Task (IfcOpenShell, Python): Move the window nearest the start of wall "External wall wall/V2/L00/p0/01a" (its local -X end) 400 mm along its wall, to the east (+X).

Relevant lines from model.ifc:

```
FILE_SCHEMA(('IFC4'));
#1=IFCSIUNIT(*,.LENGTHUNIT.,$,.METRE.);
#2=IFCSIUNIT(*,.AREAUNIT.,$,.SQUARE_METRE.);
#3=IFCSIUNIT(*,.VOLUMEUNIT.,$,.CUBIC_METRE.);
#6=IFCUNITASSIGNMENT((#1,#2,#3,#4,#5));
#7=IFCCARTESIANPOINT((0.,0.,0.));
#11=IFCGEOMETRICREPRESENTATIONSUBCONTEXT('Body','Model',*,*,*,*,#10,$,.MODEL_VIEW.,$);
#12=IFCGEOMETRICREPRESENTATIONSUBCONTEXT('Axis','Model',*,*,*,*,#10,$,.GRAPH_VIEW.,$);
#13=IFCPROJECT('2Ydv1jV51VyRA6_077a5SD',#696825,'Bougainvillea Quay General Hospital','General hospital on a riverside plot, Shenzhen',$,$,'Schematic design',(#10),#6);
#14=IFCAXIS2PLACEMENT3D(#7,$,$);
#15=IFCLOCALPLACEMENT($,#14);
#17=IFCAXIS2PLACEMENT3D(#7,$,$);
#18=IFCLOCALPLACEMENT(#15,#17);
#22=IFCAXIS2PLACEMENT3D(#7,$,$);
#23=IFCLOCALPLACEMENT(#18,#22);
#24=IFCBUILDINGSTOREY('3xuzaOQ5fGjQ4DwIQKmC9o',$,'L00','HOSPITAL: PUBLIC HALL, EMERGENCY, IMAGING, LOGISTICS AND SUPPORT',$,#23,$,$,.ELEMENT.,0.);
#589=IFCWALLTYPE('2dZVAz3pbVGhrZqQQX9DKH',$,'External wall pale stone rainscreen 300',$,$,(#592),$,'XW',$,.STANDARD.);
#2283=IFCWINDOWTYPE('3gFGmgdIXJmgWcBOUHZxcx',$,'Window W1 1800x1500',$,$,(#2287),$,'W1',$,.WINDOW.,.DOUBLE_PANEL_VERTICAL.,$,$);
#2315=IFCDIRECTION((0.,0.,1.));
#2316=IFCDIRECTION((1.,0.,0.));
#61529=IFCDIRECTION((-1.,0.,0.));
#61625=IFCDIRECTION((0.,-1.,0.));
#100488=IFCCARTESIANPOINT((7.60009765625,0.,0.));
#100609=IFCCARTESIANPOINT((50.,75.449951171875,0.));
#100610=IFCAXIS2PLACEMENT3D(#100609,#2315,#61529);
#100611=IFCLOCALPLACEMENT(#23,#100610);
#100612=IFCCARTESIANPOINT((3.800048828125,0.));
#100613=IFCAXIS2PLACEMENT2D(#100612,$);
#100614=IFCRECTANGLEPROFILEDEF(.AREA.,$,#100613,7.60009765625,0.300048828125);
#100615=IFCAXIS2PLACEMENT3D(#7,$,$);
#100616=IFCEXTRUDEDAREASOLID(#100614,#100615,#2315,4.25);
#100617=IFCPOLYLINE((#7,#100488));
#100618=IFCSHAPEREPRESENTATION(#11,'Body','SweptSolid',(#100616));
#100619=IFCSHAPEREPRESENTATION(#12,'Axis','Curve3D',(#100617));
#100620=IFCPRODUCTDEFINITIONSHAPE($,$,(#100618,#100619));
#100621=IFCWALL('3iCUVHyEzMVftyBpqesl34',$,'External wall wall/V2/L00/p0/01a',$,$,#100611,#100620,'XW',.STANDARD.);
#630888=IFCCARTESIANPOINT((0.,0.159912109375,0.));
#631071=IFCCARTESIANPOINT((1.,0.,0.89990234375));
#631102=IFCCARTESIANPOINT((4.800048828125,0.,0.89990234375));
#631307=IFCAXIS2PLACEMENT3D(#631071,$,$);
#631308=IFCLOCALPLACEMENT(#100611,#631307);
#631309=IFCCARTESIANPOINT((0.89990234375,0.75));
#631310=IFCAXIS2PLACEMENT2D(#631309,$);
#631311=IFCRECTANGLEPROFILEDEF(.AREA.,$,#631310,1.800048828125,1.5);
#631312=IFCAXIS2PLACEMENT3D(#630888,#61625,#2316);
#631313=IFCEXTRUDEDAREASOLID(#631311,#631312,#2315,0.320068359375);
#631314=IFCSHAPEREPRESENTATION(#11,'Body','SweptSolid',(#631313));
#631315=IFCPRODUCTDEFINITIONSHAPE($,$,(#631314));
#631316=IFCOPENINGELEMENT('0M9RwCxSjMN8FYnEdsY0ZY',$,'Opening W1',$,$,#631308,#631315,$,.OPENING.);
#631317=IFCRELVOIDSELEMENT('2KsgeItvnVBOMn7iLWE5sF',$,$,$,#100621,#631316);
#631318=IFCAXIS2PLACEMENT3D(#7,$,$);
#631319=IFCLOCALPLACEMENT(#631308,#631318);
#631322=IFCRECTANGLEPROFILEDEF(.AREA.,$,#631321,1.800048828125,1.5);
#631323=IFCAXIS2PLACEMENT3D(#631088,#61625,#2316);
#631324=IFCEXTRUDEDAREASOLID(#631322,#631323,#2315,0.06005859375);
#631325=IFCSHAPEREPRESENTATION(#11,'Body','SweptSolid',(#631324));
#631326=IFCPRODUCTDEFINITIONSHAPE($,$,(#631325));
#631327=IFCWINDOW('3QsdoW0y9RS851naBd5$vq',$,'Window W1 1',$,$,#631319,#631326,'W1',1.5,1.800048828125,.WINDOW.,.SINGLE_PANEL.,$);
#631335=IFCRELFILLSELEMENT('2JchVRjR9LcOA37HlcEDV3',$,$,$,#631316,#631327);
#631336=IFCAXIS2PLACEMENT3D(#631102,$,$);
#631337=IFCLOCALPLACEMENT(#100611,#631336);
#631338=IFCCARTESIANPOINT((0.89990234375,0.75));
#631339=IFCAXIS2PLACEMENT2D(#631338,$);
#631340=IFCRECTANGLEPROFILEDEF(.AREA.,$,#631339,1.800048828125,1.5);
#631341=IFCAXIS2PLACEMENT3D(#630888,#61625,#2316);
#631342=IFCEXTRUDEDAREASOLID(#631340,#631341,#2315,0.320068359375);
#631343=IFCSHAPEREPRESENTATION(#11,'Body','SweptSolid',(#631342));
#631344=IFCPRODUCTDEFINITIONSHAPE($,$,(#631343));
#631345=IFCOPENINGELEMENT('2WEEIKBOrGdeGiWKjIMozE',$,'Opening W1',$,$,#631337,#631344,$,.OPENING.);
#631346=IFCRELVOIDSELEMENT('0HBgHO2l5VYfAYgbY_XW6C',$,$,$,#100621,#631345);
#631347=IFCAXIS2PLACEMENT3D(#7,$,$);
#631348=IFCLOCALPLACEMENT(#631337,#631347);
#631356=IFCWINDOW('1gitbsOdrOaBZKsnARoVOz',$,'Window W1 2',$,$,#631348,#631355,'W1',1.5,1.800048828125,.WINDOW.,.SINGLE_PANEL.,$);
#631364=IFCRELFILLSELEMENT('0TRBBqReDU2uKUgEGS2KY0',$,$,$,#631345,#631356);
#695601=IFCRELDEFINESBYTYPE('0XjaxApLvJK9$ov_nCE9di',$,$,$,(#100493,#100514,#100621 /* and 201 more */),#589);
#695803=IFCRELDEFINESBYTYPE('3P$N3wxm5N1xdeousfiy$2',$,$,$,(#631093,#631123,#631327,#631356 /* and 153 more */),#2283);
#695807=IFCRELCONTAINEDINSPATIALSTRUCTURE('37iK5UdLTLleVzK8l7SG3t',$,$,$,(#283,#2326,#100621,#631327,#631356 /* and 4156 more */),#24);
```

```python
import ifcopenshell
import ifcopenshell.api.geometry
import ifcopenshell.util.placement

model = ifcopenshell.open("model.ifc")

window = model.by_id(631327)
opening = window.FillsVoids[0].RelatingOpeningElement
wall = opening.VoidsElements[0].RelatingBuildingElement

wall_matrix = ifcopenshell.util.placement.get_local_placement(wall.ObjectPlacement)
shift = wall_matrix[:3, 0] * -0.4
before = ifcopenshell.util.placement.get_local_placement(window.ObjectPlacement)[:3, 3].copy()

# The window is placed relative to its opening, so it follows when the opening moves.
matrix = ifcopenshell.util.placement.get_local_placement(opening.ObjectPlacement)
matrix[:3, 3] += shift
ifcopenshell.api.geometry.edit_object_placement(
    model, product=opening, matrix=matrix, is_si=False, should_transform_children=True
)

after = ifcopenshell.util.placement.get_local_placement(window.ObjectPlacement)[:3, 3]
print("window moved by", (after - before).round(3) + 0.0)

model.write("model_v2.ifc")
```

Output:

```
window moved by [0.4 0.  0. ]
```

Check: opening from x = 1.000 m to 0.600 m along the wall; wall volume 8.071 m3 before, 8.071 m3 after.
